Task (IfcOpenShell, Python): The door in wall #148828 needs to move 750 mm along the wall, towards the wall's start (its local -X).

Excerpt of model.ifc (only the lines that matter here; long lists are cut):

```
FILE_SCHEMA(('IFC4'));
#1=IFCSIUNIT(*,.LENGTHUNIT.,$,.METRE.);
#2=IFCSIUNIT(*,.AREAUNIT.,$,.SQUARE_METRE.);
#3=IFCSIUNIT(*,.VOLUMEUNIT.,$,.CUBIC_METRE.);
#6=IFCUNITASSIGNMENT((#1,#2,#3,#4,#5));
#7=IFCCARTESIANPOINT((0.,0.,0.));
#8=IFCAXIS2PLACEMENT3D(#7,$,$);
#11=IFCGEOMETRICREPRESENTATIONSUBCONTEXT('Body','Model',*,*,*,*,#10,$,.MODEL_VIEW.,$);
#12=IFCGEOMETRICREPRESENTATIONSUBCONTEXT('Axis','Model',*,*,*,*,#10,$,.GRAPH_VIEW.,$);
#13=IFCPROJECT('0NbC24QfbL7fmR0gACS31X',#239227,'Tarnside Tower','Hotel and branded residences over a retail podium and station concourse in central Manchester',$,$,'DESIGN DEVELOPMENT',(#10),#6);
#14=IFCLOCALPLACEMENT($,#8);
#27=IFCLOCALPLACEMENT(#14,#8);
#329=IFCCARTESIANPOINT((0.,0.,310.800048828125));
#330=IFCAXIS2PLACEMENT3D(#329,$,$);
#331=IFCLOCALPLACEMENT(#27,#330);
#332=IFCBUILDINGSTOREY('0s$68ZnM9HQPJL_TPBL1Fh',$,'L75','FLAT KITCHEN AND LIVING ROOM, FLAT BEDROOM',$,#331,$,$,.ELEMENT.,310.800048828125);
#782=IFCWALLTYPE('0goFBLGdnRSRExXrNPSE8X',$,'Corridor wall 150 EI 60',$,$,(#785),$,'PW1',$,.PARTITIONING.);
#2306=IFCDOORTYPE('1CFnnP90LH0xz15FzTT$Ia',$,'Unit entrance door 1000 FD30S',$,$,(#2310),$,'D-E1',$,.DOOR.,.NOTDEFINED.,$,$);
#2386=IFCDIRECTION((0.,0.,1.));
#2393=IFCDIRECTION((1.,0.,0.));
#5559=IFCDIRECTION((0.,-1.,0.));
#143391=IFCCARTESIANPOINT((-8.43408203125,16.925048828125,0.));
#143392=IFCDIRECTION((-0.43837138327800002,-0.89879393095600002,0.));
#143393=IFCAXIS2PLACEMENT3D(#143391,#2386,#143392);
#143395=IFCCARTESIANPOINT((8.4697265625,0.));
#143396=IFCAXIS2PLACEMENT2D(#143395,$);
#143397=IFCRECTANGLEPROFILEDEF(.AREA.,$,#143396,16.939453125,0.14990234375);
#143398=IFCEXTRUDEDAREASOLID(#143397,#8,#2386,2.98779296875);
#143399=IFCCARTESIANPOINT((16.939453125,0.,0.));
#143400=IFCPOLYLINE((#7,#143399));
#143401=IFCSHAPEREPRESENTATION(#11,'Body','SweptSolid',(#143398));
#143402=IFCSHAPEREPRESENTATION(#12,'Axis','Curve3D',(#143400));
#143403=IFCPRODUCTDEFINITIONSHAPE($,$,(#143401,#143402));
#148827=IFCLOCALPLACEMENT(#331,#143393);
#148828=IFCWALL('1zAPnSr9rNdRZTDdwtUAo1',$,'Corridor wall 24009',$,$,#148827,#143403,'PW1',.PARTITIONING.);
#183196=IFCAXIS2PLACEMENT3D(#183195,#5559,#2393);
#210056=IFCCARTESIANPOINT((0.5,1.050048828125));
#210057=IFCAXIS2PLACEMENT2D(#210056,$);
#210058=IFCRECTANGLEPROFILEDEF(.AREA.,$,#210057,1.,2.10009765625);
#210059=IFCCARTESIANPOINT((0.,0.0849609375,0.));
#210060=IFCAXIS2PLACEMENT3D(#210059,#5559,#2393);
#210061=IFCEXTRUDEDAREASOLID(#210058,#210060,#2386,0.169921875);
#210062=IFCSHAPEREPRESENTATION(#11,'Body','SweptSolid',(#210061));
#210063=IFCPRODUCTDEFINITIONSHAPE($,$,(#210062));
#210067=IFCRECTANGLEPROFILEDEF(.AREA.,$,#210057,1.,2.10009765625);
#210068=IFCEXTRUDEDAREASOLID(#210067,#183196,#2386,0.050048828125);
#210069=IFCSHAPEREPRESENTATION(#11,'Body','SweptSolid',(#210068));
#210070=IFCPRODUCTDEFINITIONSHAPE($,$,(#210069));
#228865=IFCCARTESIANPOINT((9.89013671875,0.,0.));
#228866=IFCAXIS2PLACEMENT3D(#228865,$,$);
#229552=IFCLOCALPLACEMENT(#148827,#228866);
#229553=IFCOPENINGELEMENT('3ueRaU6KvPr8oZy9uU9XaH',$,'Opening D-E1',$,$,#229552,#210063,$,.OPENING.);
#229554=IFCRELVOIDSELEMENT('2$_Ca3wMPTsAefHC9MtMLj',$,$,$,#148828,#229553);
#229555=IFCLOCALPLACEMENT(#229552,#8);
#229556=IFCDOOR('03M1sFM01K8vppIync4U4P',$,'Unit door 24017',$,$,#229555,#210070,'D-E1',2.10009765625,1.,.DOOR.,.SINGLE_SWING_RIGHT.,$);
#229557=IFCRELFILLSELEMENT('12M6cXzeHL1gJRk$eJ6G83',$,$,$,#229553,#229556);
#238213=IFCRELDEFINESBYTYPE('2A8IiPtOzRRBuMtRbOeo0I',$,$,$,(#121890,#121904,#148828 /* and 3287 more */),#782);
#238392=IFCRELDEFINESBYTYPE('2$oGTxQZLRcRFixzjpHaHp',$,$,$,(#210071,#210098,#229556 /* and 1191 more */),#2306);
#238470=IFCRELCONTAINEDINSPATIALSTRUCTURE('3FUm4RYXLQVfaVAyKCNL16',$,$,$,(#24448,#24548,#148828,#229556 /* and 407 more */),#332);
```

```python
import ifcopenshell
import ifcopenshell.api.geometry
import ifcopenshell.util.placement
import ifcopenshell.util.unit

model = ifcopenshell.open("model.ifc")
unit_scale = ifcopenshell.util.unit.calculate_unit_scale(model)

door = model.by_guid("03M1sFM01K8vppIync4U4P")
opening = door.FillsVoids[0].RelatingOpeningElement
wall = opening.VoidsElements[0].RelatingBuildingElement

wall_matrix = ifcopenshell.util.placement.get_local_placement(wall.ObjectPlacement)
shift = wall_matrix[:3, 0] * -0.75 / unit_scale
before = ifcopenshell.util.placement.get_local_placement(door.ObjectPlacement)[:3, 3].copy()

# The door is placed relative to its opening, so it follows when the opening moves.
matrix = ifcopenshell.util.placement.get_local_placement(opening.ObjectPlacement)
matrix[:3, 3] += shift
ifcopenshell.api.geometry.edit_object_placement(
    model, product=opening, matrix=matrix, is_si=False, should_transform_children=True
)

after = ifcopenshell.util.placement.get_local_placement(door.ObjectPlacement)[:3, 3]
print("door moved by", (after - before).round(3) + 0.0)

model.write("model_edited.ifc")
```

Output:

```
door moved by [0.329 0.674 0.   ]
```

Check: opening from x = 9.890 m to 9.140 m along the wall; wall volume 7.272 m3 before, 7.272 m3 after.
